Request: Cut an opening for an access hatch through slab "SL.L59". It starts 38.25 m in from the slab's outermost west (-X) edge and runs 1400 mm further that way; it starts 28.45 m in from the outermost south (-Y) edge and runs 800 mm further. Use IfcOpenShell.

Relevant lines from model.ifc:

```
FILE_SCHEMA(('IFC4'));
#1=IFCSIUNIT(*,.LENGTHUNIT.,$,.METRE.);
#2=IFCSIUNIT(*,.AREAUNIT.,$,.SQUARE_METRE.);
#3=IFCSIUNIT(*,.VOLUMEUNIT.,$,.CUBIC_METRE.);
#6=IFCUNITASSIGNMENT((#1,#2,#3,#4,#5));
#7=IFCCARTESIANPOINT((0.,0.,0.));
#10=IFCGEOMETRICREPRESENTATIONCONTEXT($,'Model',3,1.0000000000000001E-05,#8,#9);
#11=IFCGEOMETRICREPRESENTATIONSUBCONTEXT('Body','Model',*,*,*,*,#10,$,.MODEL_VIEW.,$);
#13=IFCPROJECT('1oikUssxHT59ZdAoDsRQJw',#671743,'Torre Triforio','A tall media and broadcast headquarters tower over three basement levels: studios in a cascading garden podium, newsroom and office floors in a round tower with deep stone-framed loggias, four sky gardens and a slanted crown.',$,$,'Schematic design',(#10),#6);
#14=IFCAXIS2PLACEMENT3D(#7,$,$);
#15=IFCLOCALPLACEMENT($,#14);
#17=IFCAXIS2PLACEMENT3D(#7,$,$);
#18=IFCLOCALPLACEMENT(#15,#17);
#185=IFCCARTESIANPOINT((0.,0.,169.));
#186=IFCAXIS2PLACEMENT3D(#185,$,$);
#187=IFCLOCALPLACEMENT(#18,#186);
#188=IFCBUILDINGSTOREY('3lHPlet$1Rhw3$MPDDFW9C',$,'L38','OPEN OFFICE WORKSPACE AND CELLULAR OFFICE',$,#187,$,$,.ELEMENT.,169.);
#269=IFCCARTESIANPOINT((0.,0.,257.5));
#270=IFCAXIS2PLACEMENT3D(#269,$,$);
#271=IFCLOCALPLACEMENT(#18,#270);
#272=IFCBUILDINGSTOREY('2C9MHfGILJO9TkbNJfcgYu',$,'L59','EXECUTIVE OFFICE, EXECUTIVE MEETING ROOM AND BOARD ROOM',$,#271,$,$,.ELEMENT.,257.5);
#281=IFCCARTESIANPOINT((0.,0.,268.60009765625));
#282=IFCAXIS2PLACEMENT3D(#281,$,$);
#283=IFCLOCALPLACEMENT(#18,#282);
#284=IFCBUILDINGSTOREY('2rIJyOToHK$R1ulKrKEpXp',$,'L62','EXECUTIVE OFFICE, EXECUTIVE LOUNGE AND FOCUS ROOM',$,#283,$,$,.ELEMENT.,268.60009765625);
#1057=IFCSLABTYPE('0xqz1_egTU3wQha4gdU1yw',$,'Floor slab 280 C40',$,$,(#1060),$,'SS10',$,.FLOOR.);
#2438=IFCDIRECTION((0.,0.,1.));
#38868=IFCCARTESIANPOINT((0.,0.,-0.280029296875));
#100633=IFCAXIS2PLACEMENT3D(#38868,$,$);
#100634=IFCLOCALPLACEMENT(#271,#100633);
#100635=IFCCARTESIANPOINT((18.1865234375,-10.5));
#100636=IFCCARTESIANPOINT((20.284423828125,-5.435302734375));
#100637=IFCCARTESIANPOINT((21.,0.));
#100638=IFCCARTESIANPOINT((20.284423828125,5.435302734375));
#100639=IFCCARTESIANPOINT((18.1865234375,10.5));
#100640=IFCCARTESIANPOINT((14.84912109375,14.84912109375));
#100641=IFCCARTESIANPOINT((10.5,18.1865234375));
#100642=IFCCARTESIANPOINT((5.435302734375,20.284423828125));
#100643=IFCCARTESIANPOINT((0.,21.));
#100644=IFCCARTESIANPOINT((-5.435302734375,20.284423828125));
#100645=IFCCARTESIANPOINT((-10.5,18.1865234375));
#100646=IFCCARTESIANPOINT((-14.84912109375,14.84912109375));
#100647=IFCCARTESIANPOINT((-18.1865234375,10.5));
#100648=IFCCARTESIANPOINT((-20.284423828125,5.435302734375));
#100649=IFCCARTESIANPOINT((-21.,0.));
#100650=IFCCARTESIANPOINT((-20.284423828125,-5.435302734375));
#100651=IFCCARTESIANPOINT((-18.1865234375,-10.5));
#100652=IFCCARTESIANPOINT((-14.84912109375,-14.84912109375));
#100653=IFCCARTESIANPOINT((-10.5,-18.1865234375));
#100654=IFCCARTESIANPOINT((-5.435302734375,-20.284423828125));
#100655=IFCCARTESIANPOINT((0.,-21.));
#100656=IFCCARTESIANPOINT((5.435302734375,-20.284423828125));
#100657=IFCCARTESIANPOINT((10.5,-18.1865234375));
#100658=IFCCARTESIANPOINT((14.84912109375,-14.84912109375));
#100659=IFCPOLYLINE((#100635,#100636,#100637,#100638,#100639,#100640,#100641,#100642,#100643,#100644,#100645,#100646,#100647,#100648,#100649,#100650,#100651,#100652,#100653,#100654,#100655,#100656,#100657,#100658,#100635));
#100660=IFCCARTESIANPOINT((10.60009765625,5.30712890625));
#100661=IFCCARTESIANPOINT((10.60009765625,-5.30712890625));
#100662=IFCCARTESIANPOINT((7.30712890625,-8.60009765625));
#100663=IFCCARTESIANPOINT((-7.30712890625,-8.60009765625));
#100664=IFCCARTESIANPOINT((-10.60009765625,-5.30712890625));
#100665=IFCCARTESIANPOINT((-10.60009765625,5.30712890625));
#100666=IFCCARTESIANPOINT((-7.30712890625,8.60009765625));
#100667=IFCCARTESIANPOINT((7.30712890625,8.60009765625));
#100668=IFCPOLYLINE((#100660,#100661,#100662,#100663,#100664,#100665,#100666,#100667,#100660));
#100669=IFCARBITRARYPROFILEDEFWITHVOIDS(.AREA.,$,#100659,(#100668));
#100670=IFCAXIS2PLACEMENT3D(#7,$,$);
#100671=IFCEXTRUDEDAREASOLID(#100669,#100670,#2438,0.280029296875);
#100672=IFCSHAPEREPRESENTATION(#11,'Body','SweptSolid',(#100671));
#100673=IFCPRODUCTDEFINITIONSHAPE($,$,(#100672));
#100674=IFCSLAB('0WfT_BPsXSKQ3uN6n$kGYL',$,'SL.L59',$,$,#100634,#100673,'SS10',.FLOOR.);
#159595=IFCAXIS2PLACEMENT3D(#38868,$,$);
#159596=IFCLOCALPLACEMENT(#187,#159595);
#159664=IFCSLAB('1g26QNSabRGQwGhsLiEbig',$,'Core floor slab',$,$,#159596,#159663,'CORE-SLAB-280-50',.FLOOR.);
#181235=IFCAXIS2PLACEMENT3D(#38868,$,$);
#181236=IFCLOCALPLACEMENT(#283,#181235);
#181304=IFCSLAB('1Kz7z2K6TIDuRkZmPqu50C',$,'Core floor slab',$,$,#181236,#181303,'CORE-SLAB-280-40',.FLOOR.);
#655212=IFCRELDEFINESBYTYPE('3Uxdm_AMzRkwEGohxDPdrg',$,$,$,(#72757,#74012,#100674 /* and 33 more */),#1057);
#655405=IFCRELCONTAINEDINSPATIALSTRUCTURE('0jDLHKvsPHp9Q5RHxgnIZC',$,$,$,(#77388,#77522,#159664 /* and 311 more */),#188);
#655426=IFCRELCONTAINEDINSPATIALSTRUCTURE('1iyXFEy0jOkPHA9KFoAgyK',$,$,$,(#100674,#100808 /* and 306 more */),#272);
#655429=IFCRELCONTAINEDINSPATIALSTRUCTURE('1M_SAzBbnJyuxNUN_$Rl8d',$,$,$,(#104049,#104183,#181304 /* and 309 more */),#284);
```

```python
import numpy as np
import ifcopenshell
import ifcopenshell.api.feature
import ifcopenshell.api.geometry
import ifcopenshell.api.root
import ifcopenshell.geom
import ifcopenshell.util.placement
import ifcopenshell.util.representation
import ifcopenshell.util.shape
import ifcopenshell.util.unit

model = ifcopenshell.open("model.ifc")
unit_scale = ifcopenshell.util.unit.calculate_unit_scale(model)
settings = ifcopenshell.geom.settings()


def volume(element):
    """Net volume in cubic metres, openings subtracted."""
    shape = ifcopenshell.geom.create_shape(settings, element)
    return ifcopenshell.util.shape.get_volume(shape.geometry)


slab = model.by_id(100674)
before = volume(slab)

# Extent in the slab's own axes, in metres. The edges named are its -X and -Y sides.
slab_shape = ifcopenshell.geom.create_shape(settings, slab)
vertices = ifcopenshell.util.shape.get_vertices(slab_shape.geometry)
x_min, y_min, bottom = vertices.min(axis=0)
top = vertices[:, 2].max()

opening = ifcopenshell.api.root.create_entity(model, ifc_class="IfcOpeningElement", name="Access hatch opening", predefined_type="OPENING")
context = ifcopenshell.util.representation.get_context(model, "Model", "Body", "MODEL_VIEW")
width, depth = 1.4, 0.8
outline = [(0.0, 0.0), (width, 0.0), (width, depth), (0.0, depth), (0.0, 0.0)]
# Overshoot both faces by 50 mm so the cut is clean.
shape = ifcopenshell.api.geometry.add_slab_representation(
    model, context=context, depth=top - bottom + 0.1, polyline=outline
)
ifcopenshell.api.geometry.assign_representation(model, product=opening, representation=shape)

matrix = ifcopenshell.util.placement.get_local_placement(slab.ObjectPlacement)
matrix[:, 3] = matrix @ np.append(np.array([x_min + 38.25, y_min + 28.45, bottom - 0.05]) / unit_scale, 1.0)
ifcopenshell.api.geometry.edit_object_placement(model, product=opening, matrix=matrix, is_si=False)
ifcopenshell.api.feature.add_feature(model, feature=opening, element=slab)

after = volume(slab)

print(f"slab volume {before:.3f} -> {after:.3f} m3")

model.write("model-out.ifc")
```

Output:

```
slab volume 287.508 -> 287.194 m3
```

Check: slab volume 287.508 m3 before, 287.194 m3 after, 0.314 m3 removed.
